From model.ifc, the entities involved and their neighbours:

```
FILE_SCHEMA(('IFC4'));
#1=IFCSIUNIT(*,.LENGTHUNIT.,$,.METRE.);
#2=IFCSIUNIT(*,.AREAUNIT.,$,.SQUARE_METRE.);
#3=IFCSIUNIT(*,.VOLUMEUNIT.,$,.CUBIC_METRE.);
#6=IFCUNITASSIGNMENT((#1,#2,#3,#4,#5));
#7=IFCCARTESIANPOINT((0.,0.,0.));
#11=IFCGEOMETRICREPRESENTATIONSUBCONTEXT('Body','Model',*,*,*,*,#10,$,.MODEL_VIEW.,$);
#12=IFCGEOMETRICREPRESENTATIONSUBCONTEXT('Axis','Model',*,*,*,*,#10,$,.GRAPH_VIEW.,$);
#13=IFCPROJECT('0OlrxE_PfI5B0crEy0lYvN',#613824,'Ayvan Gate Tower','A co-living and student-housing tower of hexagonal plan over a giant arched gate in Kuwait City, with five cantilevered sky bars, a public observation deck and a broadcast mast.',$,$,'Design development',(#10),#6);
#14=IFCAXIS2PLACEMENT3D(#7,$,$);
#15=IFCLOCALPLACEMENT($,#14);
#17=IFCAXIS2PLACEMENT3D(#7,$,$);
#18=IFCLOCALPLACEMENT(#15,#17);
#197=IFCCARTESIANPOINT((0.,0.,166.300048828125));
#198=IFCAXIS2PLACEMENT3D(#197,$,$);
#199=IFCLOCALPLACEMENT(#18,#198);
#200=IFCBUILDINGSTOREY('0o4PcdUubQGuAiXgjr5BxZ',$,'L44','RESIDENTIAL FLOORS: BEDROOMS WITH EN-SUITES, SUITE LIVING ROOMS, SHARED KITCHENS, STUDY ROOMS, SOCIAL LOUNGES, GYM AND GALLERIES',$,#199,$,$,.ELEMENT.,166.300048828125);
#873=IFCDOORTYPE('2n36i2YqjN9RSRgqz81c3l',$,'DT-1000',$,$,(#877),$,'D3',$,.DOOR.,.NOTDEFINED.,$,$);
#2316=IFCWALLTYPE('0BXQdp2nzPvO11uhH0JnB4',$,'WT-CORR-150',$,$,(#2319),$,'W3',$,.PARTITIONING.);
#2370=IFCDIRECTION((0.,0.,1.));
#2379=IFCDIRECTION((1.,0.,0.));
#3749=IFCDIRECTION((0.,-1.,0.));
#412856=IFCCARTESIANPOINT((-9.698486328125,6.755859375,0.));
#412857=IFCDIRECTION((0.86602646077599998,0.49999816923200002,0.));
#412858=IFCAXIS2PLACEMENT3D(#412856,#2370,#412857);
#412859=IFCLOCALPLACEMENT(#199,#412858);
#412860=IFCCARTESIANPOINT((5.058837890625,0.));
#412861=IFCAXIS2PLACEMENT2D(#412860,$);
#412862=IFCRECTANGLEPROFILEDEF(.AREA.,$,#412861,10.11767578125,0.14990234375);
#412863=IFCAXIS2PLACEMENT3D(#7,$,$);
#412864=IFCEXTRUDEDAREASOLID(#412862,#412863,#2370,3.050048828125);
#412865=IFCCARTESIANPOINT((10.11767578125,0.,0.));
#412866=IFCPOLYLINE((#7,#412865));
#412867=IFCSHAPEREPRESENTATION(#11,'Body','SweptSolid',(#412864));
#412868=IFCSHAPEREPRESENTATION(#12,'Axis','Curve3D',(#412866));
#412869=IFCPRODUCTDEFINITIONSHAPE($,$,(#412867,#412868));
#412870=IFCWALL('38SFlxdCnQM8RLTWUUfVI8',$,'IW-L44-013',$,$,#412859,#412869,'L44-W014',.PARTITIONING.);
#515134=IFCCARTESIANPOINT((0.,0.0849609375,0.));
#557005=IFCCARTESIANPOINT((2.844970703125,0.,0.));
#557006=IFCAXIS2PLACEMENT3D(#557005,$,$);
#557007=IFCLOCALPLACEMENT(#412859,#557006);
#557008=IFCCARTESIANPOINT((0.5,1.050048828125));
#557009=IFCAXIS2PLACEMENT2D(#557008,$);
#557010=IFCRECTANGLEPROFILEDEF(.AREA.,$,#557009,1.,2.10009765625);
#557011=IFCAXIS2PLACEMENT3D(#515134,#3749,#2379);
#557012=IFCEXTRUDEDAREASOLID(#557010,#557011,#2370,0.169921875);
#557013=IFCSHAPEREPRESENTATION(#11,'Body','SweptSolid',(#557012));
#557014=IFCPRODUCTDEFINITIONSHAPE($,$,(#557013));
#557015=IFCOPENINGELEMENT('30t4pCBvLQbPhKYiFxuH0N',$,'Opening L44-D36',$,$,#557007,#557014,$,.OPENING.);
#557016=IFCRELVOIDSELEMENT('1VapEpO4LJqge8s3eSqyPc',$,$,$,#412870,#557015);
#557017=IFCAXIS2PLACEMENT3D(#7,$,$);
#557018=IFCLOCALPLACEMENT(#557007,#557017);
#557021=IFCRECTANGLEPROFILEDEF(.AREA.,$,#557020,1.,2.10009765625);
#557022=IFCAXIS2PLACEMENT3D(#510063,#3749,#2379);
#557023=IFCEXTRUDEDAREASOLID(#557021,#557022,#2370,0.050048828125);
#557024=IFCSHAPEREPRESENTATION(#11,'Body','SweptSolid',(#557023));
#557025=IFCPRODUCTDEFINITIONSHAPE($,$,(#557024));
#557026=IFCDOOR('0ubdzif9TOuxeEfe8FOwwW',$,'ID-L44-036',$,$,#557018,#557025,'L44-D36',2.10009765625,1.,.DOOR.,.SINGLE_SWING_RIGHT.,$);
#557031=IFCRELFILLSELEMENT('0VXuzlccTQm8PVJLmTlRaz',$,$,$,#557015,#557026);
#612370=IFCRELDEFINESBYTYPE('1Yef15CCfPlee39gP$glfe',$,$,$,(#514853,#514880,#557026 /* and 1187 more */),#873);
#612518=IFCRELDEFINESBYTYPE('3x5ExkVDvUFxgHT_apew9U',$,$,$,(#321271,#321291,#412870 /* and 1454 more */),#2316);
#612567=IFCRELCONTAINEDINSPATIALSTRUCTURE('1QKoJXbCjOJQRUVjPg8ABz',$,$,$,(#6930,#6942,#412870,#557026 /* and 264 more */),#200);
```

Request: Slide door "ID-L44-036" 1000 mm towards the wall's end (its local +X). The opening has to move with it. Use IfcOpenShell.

```python
import ifcopenshell
import ifcopenshell.api.geometry
import ifcopenshell.util.placement

model = ifcopenshell.open("model.ifc")

door = model.by_guid("0ubdzif9TOuxeEfe8FOwwW")
opening = door.FillsVoids[0].RelatingOpeningElement
wall = opening.VoidsElements[0].RelatingBuildingElement

wall_matrix = ifcopenshell.util.placement.get_local_placement(wall.ObjectPlacement)
shift = wall_matrix[:3, 0] * 1.0
before = ifcopenshell.util.placement.get_local_placement(door.ObjectPlacement)[:3, 3].copy()

# The door is placed relative to its opening, so it follows when the opening moves.
matrix = ifcopenshell.util.placement.get_local_placement(opening.ObjectPlacement)
matrix[:3, 3] += shift
ifcopenshell.api.geometry.edit_object_placement(
    model, product=opening, matrix=matrix, is_si=False, should_transform_children=True
)

after = ifcopenshell.util.placement.get_local_placement(door.ObjectPlacement)[:3, 3]
print("door moved by", (after - before).round(3) + 0.0)

model.write("model_rev.ifc")
```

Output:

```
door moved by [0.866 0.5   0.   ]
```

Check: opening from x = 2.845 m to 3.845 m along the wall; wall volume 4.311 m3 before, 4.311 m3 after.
